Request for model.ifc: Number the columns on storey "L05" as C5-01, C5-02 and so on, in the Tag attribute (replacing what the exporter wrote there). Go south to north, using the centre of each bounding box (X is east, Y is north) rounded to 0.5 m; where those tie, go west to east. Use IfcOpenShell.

First a look at what the model holds.

```python
import ifcopenshell
import ifcopenshell.util.element
import ifcopenshell.util.placement

model = ifcopenshell.open("model.ifc")
print(model.schema)
storey = next(s for s in model.by_type("IfcBuildingStorey") if s.Name == "L05")
columns = [e for e in ifcopenshell.util.element.get_decomposition(storey) if e.is_a("IfcColumn")]
for e in sorted(columns, key=lambda e: e.id()):
    origin = ifcopenshell.util.placement.get_local_placement(e.ObjectPlacement)[:3, 3]
    print(e.id(), e.Tag, e.Name, origin.round(2) + 0.0, sep=" | ")
```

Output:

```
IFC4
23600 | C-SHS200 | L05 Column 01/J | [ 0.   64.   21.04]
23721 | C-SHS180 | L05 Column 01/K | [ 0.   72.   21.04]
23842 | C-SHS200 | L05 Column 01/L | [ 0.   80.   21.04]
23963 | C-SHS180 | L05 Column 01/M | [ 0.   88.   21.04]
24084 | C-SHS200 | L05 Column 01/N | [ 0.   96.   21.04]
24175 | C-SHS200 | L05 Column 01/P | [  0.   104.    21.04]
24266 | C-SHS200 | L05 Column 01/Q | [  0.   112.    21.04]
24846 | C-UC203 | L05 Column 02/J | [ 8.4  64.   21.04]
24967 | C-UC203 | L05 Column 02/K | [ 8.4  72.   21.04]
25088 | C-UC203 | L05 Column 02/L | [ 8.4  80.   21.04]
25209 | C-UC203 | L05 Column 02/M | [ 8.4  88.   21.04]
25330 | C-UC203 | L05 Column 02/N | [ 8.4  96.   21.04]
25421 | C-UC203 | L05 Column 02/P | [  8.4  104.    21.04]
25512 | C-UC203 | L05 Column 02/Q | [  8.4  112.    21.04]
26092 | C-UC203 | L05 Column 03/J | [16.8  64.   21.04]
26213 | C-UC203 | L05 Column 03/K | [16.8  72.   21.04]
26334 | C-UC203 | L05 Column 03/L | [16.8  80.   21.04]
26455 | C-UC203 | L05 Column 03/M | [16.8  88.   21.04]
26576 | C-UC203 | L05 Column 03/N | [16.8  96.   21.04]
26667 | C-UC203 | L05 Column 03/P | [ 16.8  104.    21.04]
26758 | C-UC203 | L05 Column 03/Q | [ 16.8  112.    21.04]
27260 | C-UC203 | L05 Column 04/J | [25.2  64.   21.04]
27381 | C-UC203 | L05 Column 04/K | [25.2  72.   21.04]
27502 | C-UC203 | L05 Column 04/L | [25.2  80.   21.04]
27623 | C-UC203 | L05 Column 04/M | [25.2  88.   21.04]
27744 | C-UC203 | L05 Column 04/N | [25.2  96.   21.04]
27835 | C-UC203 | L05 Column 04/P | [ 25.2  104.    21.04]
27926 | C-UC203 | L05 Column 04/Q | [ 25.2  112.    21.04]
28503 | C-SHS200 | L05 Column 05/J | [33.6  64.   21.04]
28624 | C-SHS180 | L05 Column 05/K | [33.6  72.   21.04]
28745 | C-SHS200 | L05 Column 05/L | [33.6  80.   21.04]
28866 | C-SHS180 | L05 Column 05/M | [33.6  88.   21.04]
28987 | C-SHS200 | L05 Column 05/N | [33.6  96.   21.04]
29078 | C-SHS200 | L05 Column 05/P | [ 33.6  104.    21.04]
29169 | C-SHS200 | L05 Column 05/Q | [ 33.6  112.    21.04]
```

```python
import ifcopenshell
import ifcopenshell.geom
import ifcopenshell.util.element
import ifcopenshell.util.shape

model = ifcopenshell.open("model.ifc")
settings = ifcopenshell.geom.settings()
settings.set("use-world-coords", True)


def centre(element):
    shape = ifcopenshell.geom.create_shape(settings, element)
    return ifcopenshell.util.shape.get_bbox_centroid(shape.geometry)


storey = next(s for s in model.by_type("IfcBuildingStorey") if s.Name == "L05")
columns = [e for e in ifcopenshell.util.element.get_decomposition(storey) if e.is_a("IfcColumn")]

# Insertion points can sit at a corner or the storey origin, so sort by the geometry (in metres).
centres = {e: centre(e) for e in columns}
columns.sort(key=lambda e: (round(centres[e][1] / 0.5), centres[e][0]))

for i, e in enumerate(columns, start=1):
    number = f"C5-{i:02d}"
    e.Tag = number
    print(e.id(), number)

model.write("model_edited.ifc")
```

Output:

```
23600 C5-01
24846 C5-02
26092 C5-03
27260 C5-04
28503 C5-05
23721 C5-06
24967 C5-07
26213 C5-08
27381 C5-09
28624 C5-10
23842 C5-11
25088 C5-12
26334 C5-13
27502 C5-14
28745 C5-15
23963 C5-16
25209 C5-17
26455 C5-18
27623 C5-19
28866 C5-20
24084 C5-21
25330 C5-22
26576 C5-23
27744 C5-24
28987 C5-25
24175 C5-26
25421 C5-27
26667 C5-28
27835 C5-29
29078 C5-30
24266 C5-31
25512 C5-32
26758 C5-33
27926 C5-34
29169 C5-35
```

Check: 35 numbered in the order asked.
